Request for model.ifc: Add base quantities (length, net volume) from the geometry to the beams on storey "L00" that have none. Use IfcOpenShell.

First a look at what the model holds.

```python
import ifcopenshell
import ifcopenshell.util.element
import ifcopenshell.util.unit

model = ifcopenshell.open("model.ifc")
print(model.schema)
for unit_type in ("LENGTHUNIT", "AREAUNIT", "VOLUMEUNIT"):
    print(unit_type, ifcopenshell.util.unit.calculate_unit_scale(model, unit_type))
storey = next(s for s in model.by_type("IfcBuildingStorey") if s.Name == "L00")
beams = [e for e in ifcopenshell.util.element.get_decomposition(storey) if e.is_a("IfcBeam")]
for e in sorted(beams, key=lambda e: e.id()):
    print(e.id(), e.is_a(), e.Name, list(ifcopenshell.util.element.get_psets(e, qtos_only=True)), sep=" | ")
```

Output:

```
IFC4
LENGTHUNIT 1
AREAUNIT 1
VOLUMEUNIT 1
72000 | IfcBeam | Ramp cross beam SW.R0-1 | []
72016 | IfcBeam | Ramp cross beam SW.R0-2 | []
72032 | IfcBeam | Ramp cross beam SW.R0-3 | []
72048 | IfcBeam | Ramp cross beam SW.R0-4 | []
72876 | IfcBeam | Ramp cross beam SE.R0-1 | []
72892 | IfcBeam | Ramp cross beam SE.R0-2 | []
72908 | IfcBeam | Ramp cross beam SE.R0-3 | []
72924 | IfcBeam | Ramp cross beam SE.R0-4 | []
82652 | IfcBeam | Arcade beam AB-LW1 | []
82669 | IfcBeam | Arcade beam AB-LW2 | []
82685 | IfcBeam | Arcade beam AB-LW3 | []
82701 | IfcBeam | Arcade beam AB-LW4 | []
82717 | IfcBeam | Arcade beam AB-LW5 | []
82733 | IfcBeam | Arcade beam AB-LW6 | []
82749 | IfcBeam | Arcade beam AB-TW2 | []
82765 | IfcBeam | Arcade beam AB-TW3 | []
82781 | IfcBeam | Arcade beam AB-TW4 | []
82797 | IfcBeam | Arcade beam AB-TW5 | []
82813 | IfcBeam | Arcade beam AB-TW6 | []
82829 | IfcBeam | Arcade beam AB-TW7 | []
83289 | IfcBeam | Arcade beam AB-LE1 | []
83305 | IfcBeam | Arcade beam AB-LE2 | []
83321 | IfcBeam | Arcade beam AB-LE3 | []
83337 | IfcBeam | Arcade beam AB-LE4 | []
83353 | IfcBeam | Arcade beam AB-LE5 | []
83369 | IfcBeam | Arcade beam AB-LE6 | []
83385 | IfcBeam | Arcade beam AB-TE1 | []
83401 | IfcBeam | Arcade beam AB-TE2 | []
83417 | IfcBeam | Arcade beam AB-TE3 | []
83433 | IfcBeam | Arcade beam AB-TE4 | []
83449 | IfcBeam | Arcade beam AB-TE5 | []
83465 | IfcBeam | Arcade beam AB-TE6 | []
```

```python
import ifcopenshell
import ifcopenshell.api.pset
import ifcopenshell.geom
import ifcopenshell.util.element
import ifcopenshell.util.shape
import ifcopenshell.util.unit

model = ifcopenshell.open("model.ifc")
unit_scale = ifcopenshell.util.unit.calculate_unit_scale(model)
volume_scale = ifcopenshell.util.unit.calculate_unit_scale(model, "VOLUMEUNIT")
settings = ifcopenshell.geom.settings()

storey = next(s for s in model.by_type("IfcBuildingStorey") if s.Name == "L00")
beams = [e for e in ifcopenshell.util.element.get_decomposition(storey) if e.is_a("IfcBeam")]

for e in sorted(beams, key=lambda e: e.id()):
    if ifcopenshell.util.element.get_psets(e, qtos_only=True, should_inherit=False):
        continue
    # Geometry comes back in metres, in the element's own axes.
    shape = ifcopenshell.geom.create_shape(settings, e)
    values = {
        "Length": ifcopenshell.util.shape.get_max_xyz(shape.geometry) / unit_scale,
        "NetVolume": ifcopenshell.util.shape.get_volume(shape.geometry) / volume_scale,
    }
    qto = ifcopenshell.api.pset.add_qto(model, product=e, name="Qto_BeamBaseQuantities")
    ifcopenshell.api.pset.edit_qto(model, qto=qto, properties=values)
    print(e.id(), {k: round(v, 3) for k, v in values.items()})

model.write("model_updated.ifc")
```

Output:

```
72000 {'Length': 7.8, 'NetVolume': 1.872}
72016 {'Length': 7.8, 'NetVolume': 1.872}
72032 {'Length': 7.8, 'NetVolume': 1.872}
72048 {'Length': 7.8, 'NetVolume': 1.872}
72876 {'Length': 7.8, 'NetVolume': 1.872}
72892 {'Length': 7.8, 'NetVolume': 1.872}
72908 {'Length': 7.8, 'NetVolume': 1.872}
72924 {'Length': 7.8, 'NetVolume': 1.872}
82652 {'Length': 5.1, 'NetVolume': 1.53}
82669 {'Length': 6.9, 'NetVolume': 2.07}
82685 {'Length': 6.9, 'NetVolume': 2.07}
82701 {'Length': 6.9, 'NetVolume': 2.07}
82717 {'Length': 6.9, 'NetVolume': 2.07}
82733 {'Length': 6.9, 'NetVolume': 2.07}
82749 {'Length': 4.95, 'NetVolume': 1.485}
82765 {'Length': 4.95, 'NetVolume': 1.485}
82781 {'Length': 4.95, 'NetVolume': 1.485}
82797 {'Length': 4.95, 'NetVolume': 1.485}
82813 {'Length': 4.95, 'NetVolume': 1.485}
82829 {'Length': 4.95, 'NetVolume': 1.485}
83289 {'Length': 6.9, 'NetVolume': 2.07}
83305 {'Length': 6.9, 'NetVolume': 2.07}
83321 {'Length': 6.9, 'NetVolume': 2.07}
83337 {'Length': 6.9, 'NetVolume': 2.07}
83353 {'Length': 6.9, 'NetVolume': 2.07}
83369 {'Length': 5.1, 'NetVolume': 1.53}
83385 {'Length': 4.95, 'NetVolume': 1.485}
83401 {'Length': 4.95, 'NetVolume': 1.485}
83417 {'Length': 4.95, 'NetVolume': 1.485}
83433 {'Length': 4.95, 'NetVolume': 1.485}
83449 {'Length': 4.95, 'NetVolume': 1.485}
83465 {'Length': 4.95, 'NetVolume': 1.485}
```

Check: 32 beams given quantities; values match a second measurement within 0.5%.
